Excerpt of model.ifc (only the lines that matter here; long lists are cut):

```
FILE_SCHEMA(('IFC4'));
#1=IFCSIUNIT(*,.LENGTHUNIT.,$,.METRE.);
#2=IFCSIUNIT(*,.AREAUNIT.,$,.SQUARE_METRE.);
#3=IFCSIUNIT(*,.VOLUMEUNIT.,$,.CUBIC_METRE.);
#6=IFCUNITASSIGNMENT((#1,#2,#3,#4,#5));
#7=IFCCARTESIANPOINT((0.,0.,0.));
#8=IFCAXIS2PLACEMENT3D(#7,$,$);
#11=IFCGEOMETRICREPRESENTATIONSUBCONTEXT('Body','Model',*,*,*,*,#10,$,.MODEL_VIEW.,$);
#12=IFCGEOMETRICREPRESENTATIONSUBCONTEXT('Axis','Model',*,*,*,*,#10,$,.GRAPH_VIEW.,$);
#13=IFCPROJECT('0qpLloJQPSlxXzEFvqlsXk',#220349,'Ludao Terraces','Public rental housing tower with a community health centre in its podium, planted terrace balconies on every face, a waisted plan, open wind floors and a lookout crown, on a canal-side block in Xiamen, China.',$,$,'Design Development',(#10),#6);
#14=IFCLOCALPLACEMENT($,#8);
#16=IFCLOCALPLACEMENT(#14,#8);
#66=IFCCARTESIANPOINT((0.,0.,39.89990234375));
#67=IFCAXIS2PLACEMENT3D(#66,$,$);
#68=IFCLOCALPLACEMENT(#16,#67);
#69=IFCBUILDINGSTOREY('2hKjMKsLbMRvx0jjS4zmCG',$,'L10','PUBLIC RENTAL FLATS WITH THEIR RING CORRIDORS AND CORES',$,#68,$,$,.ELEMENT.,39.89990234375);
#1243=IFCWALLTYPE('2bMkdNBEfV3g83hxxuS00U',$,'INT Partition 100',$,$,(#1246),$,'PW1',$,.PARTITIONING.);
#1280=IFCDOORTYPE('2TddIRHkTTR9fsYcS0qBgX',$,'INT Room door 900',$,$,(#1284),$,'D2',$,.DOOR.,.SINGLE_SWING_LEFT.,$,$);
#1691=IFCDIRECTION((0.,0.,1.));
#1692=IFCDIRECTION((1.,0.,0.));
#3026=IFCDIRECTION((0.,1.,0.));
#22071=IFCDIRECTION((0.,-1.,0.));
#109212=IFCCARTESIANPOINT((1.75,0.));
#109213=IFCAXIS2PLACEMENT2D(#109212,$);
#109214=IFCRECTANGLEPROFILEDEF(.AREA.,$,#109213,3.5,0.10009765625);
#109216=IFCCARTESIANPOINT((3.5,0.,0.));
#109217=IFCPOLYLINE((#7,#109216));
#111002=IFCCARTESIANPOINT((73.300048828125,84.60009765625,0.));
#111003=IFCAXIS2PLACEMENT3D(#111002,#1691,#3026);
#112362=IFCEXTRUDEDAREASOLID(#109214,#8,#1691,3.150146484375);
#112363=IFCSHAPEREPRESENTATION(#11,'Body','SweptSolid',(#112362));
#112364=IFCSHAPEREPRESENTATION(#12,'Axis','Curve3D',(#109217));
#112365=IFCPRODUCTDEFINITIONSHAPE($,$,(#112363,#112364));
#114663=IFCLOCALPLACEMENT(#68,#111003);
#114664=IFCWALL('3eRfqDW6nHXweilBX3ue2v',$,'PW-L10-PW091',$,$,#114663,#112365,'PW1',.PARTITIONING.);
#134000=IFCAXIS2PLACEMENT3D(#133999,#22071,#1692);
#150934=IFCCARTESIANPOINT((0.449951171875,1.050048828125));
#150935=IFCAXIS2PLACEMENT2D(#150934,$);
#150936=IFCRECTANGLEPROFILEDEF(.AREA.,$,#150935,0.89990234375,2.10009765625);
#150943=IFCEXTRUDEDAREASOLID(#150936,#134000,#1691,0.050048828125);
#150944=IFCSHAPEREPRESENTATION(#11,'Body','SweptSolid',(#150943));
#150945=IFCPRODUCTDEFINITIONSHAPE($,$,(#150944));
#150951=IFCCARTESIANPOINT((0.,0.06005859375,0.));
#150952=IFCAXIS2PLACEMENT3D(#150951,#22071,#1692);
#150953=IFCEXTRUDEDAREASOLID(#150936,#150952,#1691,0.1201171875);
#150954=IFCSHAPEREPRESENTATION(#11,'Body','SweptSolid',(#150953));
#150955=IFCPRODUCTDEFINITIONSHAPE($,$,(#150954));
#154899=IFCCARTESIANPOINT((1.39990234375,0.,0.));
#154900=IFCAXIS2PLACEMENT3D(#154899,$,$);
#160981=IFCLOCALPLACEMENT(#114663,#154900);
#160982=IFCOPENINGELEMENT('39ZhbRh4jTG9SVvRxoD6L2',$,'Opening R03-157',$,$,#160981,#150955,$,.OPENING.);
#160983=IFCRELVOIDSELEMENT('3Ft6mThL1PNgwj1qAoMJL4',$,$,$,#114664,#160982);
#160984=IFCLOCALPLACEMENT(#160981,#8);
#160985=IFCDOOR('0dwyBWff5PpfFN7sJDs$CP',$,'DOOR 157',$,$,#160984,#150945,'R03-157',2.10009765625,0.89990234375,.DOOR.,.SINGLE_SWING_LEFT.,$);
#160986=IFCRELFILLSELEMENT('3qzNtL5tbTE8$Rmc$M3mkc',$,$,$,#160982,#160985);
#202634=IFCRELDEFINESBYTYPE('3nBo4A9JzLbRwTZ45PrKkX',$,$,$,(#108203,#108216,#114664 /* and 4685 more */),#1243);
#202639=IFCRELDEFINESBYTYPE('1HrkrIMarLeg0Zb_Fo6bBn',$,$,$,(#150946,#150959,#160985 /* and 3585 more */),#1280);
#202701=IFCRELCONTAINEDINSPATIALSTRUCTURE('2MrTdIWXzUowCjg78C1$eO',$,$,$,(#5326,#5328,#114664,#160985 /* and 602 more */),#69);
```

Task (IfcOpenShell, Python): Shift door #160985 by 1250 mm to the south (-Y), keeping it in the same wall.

```python
import ifcopenshell
import ifcopenshell.api.geometry
import ifcopenshell.util.placement
import ifcopenshell.util.unit

model = ifcopenshell.open("model.ifc")
unit_scale = ifcopenshell.util.unit.calculate_unit_scale(model)

door = model.by_guid("0dwyBWff5PpfFN7sJDs$CP")
opening = door.FillsVoids[0].RelatingOpeningElement
wall = opening.VoidsElements[0].RelatingBuildingElement

wall_matrix = ifcopenshell.util.placement.get_local_placement(wall.ObjectPlacement)
shift = wall_matrix[:3, 0] * -1.25 / unit_scale
before = ifcopenshell.util.placement.get_local_placement(door.ObjectPlacement)[:3, 3].copy()

# The door is placed relative to its opening, so it follows when the opening moves.
matrix = ifcopenshell.util.placement.get_local_placement(opening.ObjectPlacement)
matrix[:3, 3] += shift
ifcopenshell.api.geometry.edit_object_placement(
    model, product=opening, matrix=matrix, is_si=False, should_transform_children=True
)

after = ifcopenshell.util.placement.get_local_placement(door.ObjectPlacement)[:3, 3]
print("door moved by", (after - before).round(3) + 0.0)

model.write("model-out.ifc")
```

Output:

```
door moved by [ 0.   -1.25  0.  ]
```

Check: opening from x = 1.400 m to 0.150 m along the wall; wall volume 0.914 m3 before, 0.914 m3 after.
